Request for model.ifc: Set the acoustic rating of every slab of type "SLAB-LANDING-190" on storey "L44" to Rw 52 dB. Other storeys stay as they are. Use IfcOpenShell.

First a look at what the model holds.

```python
import ifcopenshell
import ifcopenshell.util.element

model = ifcopenshell.open("model.ifc")
print(model.schema)
storey = next(s for s in model.by_type("IfcBuildingStorey") if s.Name == "L44")
slabs = [e for e in ifcopenshell.util.element.get_decomposition(storey) if e.is_a("IfcSlab")]
seen = {}
for e in slabs:
    element_type = ifcopenshell.util.element.get_type(e)
    key = (element_type.Name if element_type != e and element_type else None, ifcopenshell.util.element.get_pset(e, "Pset_SlabCommon", "AcousticRating"))
    seen[key] = seen.get(key, 0) + 1
for (name, value), count in sorted(seen.items(), key=str):
    print(count, "x", name, "|", value)
```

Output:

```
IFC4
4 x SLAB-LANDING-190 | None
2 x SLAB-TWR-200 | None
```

```python
import ifcopenshell
import ifcopenshell.api.pset
import ifcopenshell.util.element

model = ifcopenshell.open("model.ifc")

storey = next(s for s in model.by_type("IfcBuildingStorey") if s.Name == "L44")
slabs = [e for e in ifcopenshell.util.element.get_decomposition(storey) if e.is_a("IfcSlab")]

count = 0
for e in slabs:
    element_type = ifcopenshell.util.element.get_type(e)
    if element_type in (None, e) or element_type.Name != "SLAB-LANDING-190":
        continue
    found = ifcopenshell.util.element.get_pset(e, "Pset_SlabCommon", should_inherit=False)
    if found:
        pset = model.by_id(found["id"])
        if len(ifcopenshell.util.element.get_elements_by_pset(pset)) > 1:
            pset = ifcopenshell.api.pset.unshare_pset(model, products=[e], pset=pset)[0]
    else:
        pset = ifcopenshell.api.pset.add_pset(model, product=e, name="Pset_SlabCommon")
    ifcopenshell.api.pset.edit_pset(model, pset=pset, properties={"AcousticRating": "Rw 52 dB"})
    count += 1

print(count, "slabs updated")

model.write("model-out.ifc")
```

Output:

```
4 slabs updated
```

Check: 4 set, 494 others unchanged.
